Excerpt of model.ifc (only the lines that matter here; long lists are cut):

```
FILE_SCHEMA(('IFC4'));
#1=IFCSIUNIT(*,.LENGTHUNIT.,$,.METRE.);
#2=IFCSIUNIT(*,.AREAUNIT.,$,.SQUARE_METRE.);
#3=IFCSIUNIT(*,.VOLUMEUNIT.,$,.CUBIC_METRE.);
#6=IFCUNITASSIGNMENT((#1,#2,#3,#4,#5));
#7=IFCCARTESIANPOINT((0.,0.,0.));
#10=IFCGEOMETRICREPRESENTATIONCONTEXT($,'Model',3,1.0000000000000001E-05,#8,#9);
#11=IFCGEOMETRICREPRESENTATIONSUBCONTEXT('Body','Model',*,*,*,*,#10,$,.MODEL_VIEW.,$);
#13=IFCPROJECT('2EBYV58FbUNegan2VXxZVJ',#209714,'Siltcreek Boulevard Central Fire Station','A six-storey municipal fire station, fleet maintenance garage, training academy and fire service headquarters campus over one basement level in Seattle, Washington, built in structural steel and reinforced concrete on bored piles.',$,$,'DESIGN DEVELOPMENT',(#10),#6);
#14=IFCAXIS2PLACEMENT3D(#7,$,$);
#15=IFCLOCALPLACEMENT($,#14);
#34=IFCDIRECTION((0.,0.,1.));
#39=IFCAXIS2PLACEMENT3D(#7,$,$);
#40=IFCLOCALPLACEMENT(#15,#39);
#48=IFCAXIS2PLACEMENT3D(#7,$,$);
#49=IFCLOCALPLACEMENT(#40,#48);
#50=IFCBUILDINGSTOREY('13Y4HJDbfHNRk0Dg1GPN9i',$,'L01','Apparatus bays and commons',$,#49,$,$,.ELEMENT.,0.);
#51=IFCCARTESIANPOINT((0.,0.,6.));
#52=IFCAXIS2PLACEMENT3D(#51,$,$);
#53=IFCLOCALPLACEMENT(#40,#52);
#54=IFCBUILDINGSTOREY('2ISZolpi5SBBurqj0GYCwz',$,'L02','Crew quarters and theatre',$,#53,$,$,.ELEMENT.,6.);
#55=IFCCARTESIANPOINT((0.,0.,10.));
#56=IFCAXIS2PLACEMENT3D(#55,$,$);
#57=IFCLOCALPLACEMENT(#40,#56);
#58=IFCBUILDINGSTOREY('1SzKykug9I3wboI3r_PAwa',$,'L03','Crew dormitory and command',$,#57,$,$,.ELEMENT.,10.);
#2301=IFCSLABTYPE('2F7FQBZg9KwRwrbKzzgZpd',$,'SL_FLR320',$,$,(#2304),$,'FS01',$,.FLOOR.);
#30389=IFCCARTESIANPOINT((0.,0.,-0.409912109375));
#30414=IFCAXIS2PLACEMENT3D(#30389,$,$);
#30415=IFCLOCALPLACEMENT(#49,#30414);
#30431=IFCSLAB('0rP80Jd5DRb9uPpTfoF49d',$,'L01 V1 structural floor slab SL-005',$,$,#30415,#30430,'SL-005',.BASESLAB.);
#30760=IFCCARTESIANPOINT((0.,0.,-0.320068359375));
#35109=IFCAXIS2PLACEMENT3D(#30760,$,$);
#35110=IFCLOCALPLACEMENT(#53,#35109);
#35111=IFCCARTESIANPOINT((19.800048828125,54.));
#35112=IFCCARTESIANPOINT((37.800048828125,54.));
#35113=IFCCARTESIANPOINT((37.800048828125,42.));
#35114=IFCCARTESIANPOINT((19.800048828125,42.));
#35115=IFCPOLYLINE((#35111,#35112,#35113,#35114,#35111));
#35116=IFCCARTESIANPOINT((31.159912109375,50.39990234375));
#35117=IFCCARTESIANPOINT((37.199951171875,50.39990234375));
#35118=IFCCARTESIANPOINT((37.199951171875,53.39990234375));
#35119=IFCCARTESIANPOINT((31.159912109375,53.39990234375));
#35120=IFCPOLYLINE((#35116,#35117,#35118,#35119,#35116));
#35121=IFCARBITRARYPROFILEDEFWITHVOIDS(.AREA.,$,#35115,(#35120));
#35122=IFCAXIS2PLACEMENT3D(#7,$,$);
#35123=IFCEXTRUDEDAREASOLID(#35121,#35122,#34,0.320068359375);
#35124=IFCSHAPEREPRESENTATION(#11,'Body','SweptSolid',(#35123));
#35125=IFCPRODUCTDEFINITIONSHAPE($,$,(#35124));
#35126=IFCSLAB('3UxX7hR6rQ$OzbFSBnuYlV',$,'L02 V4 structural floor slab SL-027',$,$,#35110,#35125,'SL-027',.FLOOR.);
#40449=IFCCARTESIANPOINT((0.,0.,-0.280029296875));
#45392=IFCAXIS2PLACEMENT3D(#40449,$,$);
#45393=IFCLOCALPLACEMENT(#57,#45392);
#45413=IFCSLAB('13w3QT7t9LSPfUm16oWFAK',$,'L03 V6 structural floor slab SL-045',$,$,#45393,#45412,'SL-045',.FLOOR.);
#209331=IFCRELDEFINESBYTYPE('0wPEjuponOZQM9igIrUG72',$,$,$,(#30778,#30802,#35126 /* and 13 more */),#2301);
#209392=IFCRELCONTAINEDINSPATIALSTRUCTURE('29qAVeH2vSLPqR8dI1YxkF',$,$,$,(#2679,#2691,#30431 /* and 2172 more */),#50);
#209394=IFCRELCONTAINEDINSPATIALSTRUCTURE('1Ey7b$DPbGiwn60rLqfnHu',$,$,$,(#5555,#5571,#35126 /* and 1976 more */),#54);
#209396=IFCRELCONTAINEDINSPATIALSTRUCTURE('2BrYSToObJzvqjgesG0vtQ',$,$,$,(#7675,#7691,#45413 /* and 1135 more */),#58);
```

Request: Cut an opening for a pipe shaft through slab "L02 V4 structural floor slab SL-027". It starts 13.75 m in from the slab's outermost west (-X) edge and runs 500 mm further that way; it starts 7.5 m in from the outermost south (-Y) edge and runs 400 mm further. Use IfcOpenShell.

```python
import numpy as np
import ifcopenshell
import ifcopenshell.api.feature
import ifcopenshell.api.geometry
import ifcopenshell.api.root
import ifcopenshell.geom
import ifcopenshell.util.placement
import ifcopenshell.util.representation
import ifcopenshell.util.shape
import ifcopenshell.util.unit

model = ifcopenshell.open("model.ifc")
unit_scale = ifcopenshell.util.unit.calculate_unit_scale(model)
settings = ifcopenshell.geom.settings()


def volume(element):
    """Net volume in cubic metres, openings subtracted."""
    shape = ifcopenshell.geom.create_shape(settings, element)
    return ifcopenshell.util.shape.get_volume(shape.geometry)


slab = model.by_id(35126)
before = volume(slab)

# Extent in the slab's own axes, in metres. The edges named are its -X and -Y sides.
slab_shape = ifcopenshell.geom.create_shape(settings, slab)
vertices = ifcopenshell.util.shape.get_vertices(slab_shape.geometry)
x_min, y_min, bottom = vertices.min(axis=0)
top = vertices[:, 2].max()

opening = ifcopenshell.api.root.create_entity(model, ifc_class="IfcOpeningElement", name="Pipe shaft opening", predefined_type="OPENING")
context = ifcopenshell.util.representation.get_context(model, "Model", "Body", "MODEL_VIEW")
width, depth = 0.5, 0.4
outline = [(0.0, 0.0), (width, 0.0), (width, depth), (0.0, depth), (0.0, 0.0)]
# Overshoot both faces by 50 mm so the cut is clean.
shape = ifcopenshell.api.geometry.add_slab_representation(
    model, context=context, depth=top - bottom + 0.1, polyline=outline
)
ifcopenshell.api.geometry.assign_representation(model, product=opening, representation=shape)

matrix = ifcopenshell.util.placement.get_local_placement(slab.ObjectPlacement)
matrix[:, 3] = matrix @ np.append(np.array([x_min + 13.75, y_min + 7.5, bottom - 0.05]) / unit_scale, 1.0)
ifcopenshell.api.geometry.edit_object_placement(model, product=opening, matrix=matrix, is_si=False)
ifcopenshell.api.feature.add_feature(model, feature=opening, element=slab)

after = volume(slab)

print(f"slab volume {before:.3f} -> {after:.3f} m3")

model.write("model-out.ifc")
```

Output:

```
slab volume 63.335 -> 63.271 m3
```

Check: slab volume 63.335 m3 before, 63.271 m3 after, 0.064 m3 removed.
